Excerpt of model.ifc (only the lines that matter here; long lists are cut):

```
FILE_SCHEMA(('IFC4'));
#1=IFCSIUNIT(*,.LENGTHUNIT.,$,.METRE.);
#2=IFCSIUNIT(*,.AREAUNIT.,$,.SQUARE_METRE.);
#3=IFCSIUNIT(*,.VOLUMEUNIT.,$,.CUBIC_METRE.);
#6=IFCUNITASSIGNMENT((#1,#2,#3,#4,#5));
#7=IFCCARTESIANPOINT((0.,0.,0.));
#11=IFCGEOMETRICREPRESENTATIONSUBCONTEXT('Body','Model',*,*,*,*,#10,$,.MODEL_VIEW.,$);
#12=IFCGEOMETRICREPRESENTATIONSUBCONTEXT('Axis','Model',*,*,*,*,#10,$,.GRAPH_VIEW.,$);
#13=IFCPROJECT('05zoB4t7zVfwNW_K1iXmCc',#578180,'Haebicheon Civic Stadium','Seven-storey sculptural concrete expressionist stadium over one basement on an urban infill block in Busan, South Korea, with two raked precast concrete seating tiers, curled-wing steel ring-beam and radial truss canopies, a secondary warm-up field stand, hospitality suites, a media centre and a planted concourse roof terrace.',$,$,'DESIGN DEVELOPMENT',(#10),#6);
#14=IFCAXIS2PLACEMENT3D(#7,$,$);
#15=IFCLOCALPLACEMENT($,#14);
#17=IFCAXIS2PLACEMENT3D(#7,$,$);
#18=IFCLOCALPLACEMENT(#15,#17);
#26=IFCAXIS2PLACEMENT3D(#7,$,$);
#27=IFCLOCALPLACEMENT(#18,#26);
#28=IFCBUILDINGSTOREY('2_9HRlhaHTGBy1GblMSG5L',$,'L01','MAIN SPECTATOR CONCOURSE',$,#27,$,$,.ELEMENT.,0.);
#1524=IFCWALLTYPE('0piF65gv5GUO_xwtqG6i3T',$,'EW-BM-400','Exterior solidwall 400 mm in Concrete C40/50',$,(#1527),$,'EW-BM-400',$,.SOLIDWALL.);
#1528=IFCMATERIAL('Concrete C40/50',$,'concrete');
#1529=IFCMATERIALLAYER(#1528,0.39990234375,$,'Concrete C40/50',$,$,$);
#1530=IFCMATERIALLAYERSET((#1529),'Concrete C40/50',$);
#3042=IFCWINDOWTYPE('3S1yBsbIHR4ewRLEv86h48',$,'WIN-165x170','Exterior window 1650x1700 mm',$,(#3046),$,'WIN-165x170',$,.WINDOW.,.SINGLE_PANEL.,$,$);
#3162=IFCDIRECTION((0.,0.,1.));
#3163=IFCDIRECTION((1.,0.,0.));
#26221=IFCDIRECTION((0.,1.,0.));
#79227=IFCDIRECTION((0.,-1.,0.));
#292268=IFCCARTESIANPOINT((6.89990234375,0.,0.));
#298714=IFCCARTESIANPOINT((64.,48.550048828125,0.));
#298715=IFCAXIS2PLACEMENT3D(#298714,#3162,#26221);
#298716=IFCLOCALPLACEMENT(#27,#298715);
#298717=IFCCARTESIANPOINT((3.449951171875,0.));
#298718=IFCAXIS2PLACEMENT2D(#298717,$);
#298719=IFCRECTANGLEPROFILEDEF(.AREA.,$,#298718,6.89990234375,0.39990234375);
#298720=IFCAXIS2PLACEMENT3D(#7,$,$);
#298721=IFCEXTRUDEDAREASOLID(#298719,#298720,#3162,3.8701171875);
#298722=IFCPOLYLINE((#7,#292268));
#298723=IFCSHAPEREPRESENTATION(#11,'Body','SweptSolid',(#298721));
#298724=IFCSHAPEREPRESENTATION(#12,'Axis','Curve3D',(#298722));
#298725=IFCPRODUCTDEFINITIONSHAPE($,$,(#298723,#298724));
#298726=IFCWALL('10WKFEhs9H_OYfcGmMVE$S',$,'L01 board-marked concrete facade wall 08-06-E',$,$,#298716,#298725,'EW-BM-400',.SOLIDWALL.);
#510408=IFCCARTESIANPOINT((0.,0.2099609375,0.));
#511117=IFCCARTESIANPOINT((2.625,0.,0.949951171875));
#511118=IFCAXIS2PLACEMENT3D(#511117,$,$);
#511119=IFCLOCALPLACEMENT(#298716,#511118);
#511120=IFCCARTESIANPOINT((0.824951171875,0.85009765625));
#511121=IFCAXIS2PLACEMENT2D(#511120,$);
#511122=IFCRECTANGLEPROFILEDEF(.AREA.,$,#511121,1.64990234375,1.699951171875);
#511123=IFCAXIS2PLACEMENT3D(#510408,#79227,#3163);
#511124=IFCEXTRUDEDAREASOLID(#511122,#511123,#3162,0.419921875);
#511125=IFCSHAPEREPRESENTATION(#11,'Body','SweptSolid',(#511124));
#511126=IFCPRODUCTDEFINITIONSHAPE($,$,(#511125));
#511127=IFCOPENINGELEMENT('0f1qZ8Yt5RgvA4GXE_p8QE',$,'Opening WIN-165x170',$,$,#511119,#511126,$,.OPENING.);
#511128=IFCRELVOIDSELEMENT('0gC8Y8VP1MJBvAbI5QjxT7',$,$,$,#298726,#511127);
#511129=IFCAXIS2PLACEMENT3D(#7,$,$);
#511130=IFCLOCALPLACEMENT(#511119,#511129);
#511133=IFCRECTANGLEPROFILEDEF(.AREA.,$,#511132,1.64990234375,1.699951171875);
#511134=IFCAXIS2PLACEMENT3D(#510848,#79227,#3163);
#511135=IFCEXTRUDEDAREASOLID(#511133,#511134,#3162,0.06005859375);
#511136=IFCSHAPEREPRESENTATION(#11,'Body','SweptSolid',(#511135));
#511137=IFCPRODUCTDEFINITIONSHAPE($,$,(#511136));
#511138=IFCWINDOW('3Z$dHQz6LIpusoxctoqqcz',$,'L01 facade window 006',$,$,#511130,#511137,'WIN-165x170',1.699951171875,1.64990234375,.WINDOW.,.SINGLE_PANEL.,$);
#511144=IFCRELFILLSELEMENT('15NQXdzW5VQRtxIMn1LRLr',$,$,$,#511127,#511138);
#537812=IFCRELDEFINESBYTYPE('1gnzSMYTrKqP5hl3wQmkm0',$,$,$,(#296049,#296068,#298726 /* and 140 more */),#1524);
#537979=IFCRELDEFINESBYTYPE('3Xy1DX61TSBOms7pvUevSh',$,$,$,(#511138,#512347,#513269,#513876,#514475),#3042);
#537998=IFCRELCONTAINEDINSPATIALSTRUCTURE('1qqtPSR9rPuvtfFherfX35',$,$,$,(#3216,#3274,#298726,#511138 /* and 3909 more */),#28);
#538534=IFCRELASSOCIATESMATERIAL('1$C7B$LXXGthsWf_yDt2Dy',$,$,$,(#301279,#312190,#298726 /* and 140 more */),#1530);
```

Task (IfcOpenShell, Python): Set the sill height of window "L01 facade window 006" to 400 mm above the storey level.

```python
import numpy as np
import ifcopenshell
import ifcopenshell.api.geometry
import ifcopenshell.geom
import ifcopenshell.util.element
import ifcopenshell.util.placement
import ifcopenshell.util.shape
import ifcopenshell.util.unit

model = ifcopenshell.open("model.ifc")
unit_scale = ifcopenshell.util.unit.calculate_unit_scale(model)

window = model.by_id(511138)
opening = window.FillsVoids[0].RelatingOpeningElement
storey = ifcopenshell.util.element.get_container(window, ifc_class="IfcBuildingStorey")
level = ifcopenshell.util.placement.get_local_placement(storey.ObjectPlacement)[2, 3]

# The opening's origin need not be at the sill, so measure its lowest point.
shape = ifcopenshell.geom.create_shape(ifcopenshell.geom.settings(), opening)
bottom = ifcopenshell.util.shape.get_shape_bottom_elevation(shape, shape.geometry) / unit_scale
dz = level + 0.4 / unit_scale - bottom

shift = np.array([0.0, 0.0, dz])
# The window is placed relative to its opening, so it follows when the opening moves.
matrix = ifcopenshell.util.placement.get_local_placement(opening.ObjectPlacement)
matrix[:3, 3] += shift
ifcopenshell.api.geometry.edit_object_placement(
    model, product=opening, matrix=matrix, is_si=False, should_transform_children=True
)

print(f"moved by {dz * unit_scale:+.3f} m")

model.write("model_v2.ifc")
```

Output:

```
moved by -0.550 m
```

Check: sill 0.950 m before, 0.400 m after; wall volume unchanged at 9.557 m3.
